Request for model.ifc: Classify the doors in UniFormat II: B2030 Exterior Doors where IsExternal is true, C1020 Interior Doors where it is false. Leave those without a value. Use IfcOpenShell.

First a look at what the model holds.

```python
import ifcopenshell
import ifcopenshell.util.element

model = ifcopenshell.open("model.ifc")
print(model.schema)
print("classifications:", [c.Name for c in model.by_type("IfcClassification")])
values = [ifcopenshell.util.element.get_pset(e, "Pset_DoorCommon", "IsExternal") for e in model.by_type("IfcDoor")]
for value in (True, False, None):
    print("IsExternal", value, values.count(value))
```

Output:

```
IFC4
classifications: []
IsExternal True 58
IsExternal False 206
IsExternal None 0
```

```python
import ifcopenshell
import ifcopenshell.api.classification
import ifcopenshell.util.element

model = ifcopenshell.open("model.ifc")

system = ifcopenshell.api.classification.add_classification(model, classification="UniFormat II")

doors = model.by_type("IfcDoor")
external = {e: ifcopenshell.util.element.get_pset(e, "Pset_DoorCommon", "IsExternal") for e in doors}
for flag, code, name in ((True, "B2030", "Exterior Doors"), (False, "C1020", "Interior Doors")):
    products = [e for e in doors if external[e] is flag]
    ifcopenshell.api.classification.add_reference(
        model, products=products, classification=system, identification=code, name=name
    )
    print(code, len(products))

model.write("model_updated.ifc")
```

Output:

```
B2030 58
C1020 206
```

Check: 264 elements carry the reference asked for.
